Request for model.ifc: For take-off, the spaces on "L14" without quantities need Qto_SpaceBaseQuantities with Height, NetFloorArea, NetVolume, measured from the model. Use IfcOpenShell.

First a look at what the model holds.

```python
import ifcopenshell
import ifcopenshell.util.element
import ifcopenshell.util.unit

model = ifcopenshell.open("model.ifc")
print(model.schema)
for unit_type in ("LENGTHUNIT", "AREAUNIT", "VOLUMEUNIT"):
    print(unit_type, ifcopenshell.util.unit.calculate_unit_scale(model, unit_type))
storey = next(s for s in model.by_type("IfcBuildingStorey") if s.Name == "L14")
spaces = [e for e in ifcopenshell.util.element.get_decomposition(storey) if e.is_a("IfcSpace")]
for e in sorted(spaces, key=lambda e: e.id()):
    print(e.id(), e.is_a(), e.Name, list(ifcopenshell.util.element.get_psets(e, qtos_only=True)), sep=" | ")
```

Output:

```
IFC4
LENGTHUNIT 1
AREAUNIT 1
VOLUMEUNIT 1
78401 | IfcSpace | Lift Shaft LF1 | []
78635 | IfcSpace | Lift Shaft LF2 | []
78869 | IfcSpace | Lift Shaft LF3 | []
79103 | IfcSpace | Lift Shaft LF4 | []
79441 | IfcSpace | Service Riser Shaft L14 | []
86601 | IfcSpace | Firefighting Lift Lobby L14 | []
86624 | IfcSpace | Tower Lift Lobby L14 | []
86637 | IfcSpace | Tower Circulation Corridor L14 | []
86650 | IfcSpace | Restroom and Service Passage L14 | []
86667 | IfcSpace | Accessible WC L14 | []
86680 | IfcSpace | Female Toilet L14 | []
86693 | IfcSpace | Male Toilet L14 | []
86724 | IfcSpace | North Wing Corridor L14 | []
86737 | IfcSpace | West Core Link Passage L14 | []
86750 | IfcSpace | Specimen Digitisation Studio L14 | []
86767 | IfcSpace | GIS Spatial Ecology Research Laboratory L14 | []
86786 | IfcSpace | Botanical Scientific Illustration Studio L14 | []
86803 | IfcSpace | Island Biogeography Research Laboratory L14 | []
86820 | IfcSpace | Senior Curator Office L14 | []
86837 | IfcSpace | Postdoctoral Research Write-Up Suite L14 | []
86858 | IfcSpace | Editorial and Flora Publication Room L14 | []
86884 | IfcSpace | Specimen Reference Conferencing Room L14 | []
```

```python
import ifcopenshell
import ifcopenshell.api.pset
import ifcopenshell.geom
import ifcopenshell.util.element
import ifcopenshell.util.shape
import ifcopenshell.util.unit

model = ifcopenshell.open("model.ifc")
unit_scale = ifcopenshell.util.unit.calculate_unit_scale(model)
area_scale = ifcopenshell.util.unit.calculate_unit_scale(model, "AREAUNIT")
volume_scale = ifcopenshell.util.unit.calculate_unit_scale(model, "VOLUMEUNIT")
settings = ifcopenshell.geom.settings()

storey = next(s for s in model.by_type("IfcBuildingStorey") if s.Name == "L14")
spaces = [e for e in ifcopenshell.util.element.get_decomposition(storey) if e.is_a("IfcSpace")]

for e in sorted(spaces, key=lambda e: e.id()):
    if ifcopenshell.util.element.get_psets(e, qtos_only=True, should_inherit=False):
        continue
    # Geometry comes back in metres, in the element's own axes.
    shape = ifcopenshell.geom.create_shape(settings, e)
    values = {
        "Height": ifcopenshell.util.shape.get_z(shape.geometry) / unit_scale,
        "NetFloorArea": ifcopenshell.util.shape.get_footprint_area(shape.geometry) / area_scale,
        "NetVolume": ifcopenshell.util.shape.get_volume(shape.geometry) / volume_scale,
    }
    qto = ifcopenshell.api.pset.add_qto(model, product=e, name="Qto_SpaceBaseQuantities")
    ifcopenshell.api.pset.edit_qto(model, qto=qto, properties=values)
    print(e.id(), {k: round(v, 3) for k, v in values.items()})

model.write("model_updated.ifc")
```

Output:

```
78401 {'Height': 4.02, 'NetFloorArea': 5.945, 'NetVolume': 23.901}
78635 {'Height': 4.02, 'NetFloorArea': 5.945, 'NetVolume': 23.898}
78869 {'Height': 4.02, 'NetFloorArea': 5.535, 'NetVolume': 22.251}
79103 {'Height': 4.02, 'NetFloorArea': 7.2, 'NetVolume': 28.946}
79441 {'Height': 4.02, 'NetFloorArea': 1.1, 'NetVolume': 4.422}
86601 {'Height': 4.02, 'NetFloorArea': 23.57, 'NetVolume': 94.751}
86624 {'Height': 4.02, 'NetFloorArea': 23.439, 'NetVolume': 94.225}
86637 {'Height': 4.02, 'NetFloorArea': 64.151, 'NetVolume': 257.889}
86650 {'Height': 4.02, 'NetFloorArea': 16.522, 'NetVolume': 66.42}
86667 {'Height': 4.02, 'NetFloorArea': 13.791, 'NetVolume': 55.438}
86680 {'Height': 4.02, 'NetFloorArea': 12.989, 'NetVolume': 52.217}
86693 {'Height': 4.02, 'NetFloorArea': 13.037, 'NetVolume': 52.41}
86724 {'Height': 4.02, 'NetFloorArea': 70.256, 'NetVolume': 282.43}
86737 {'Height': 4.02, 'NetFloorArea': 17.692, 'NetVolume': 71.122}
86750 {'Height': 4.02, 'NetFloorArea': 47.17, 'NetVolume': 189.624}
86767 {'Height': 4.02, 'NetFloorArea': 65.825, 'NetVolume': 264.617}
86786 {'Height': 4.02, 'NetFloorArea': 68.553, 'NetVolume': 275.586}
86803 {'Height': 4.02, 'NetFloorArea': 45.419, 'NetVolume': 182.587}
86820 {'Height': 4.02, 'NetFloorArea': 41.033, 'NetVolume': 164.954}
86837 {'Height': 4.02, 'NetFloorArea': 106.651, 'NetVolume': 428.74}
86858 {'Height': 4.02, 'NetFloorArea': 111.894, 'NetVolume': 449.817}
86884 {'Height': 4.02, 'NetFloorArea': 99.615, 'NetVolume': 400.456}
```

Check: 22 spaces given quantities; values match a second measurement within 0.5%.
